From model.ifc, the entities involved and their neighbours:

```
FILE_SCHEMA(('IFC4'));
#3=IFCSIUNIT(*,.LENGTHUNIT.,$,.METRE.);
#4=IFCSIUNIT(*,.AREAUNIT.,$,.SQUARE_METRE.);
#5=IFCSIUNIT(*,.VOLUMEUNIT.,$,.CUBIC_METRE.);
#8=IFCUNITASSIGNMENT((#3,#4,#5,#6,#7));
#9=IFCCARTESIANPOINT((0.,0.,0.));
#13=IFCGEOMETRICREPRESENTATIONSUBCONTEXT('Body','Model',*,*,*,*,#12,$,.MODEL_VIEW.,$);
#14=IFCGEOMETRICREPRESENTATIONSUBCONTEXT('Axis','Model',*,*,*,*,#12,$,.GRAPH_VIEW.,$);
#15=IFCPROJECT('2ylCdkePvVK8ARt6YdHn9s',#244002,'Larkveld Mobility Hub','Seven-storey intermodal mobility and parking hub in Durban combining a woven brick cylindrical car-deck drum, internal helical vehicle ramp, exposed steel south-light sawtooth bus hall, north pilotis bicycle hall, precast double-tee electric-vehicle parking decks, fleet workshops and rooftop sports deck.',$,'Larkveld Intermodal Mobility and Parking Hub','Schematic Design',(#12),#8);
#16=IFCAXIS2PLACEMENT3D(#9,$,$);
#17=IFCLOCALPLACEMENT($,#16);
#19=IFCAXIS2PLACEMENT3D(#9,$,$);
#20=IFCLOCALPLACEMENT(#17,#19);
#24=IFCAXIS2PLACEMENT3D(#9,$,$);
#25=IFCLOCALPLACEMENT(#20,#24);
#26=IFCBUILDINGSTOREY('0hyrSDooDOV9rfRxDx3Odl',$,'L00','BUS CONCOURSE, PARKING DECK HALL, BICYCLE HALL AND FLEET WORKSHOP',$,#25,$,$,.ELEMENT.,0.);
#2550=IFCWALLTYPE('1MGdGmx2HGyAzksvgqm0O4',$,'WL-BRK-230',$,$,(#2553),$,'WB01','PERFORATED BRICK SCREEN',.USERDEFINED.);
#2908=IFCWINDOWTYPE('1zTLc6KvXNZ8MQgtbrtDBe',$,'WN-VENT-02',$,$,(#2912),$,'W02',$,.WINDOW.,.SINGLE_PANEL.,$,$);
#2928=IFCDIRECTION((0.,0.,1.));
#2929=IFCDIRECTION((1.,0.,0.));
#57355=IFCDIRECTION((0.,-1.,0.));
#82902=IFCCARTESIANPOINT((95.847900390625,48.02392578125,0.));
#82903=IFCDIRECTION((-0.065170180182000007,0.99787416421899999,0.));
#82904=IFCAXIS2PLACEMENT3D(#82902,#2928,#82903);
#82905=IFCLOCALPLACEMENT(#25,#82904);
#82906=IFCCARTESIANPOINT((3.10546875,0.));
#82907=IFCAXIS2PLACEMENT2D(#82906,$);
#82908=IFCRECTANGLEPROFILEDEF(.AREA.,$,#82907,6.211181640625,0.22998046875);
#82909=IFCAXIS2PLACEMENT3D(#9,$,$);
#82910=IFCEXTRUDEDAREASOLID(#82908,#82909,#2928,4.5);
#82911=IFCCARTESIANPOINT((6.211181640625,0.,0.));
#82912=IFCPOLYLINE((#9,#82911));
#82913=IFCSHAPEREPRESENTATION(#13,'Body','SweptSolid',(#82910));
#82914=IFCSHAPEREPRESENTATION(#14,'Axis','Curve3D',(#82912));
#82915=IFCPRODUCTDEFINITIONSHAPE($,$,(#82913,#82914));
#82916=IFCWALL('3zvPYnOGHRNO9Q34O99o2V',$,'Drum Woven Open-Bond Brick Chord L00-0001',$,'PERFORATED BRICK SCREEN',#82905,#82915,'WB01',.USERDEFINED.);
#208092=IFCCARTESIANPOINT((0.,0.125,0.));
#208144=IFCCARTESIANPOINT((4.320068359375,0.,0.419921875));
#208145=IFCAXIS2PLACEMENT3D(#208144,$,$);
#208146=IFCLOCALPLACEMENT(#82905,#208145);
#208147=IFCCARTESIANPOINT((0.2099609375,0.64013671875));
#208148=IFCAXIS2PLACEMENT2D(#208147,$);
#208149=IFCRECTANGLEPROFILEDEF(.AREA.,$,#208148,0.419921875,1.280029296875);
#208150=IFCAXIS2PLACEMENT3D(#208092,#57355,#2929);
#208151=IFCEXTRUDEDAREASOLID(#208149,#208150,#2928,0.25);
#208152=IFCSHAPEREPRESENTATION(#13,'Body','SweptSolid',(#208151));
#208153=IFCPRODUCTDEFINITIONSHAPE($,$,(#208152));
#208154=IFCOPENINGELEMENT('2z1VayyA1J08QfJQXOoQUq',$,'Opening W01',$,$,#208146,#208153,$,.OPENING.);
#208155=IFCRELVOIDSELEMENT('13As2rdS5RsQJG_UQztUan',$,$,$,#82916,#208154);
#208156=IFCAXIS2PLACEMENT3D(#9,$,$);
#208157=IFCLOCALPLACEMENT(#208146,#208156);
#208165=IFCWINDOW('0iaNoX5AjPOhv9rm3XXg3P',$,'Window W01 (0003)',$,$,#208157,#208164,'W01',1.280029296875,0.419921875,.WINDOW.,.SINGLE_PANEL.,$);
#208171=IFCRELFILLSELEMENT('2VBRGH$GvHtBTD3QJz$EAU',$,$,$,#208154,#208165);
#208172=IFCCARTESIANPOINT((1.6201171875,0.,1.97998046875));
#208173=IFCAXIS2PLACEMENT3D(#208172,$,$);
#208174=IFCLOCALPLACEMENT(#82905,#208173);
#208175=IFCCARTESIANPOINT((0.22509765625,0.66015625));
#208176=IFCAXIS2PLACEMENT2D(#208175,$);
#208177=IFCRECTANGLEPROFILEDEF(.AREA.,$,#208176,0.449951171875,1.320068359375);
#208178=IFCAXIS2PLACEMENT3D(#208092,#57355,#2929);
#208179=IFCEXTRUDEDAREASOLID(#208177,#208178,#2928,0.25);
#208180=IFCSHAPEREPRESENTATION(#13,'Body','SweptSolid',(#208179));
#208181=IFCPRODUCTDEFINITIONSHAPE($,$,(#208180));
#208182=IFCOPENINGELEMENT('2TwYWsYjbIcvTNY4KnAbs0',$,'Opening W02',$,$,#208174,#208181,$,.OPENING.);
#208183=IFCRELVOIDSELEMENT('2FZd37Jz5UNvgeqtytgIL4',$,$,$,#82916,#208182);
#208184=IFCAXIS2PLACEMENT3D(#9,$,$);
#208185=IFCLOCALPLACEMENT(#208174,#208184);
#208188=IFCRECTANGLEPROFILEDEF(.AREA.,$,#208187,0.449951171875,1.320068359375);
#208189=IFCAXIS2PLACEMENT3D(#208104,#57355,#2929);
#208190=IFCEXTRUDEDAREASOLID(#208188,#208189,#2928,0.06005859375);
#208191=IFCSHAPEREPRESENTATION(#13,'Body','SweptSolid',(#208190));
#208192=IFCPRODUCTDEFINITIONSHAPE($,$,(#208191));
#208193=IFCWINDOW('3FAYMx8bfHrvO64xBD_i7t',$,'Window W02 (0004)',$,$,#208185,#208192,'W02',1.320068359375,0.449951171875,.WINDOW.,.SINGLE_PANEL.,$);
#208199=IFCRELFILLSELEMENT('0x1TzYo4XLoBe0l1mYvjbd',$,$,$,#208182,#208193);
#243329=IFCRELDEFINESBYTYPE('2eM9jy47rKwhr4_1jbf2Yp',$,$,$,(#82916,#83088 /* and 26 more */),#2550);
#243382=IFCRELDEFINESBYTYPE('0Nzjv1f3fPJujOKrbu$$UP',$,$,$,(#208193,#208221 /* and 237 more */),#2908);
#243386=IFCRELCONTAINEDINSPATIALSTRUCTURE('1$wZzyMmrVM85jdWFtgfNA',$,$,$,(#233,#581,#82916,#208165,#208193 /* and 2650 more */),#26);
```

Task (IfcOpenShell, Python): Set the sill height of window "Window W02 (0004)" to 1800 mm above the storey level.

```python
import numpy as np
import ifcopenshell
import ifcopenshell.api.geometry
import ifcopenshell.geom
import ifcopenshell.util.element
import ifcopenshell.util.placement
import ifcopenshell.util.shape
import ifcopenshell.util.unit

model = ifcopenshell.open("model.ifc")
unit_scale = ifcopenshell.util.unit.calculate_unit_scale(model)

window = model.by_guid("3FAYMx8bfHrvO64xBD_i7t")
opening = window.FillsVoids[0].RelatingOpeningElement
storey = ifcopenshell.util.element.get_container(window, ifc_class="IfcBuildingStorey")
level = ifcopenshell.util.placement.get_local_placement(storey.ObjectPlacement)[2, 3]

# The opening's origin need not be at the sill, so measure its lowest point.
shape = ifcopenshell.geom.create_shape(ifcopenshell.geom.settings(), opening)
bottom = ifcopenshell.util.shape.get_shape_bottom_elevation(shape, shape.geometry) / unit_scale
dz = level + 1.8 - bottom

shift = np.array([0.0, 0.0, dz])
# The window is placed relative to its opening, so it follows when the opening moves.
matrix = ifcopenshell.util.placement.get_local_placement(opening.ObjectPlacement)
matrix[:3, 3] += shift
ifcopenshell.api.geometry.edit_object_placement(
    model, product=opening, matrix=matrix, is_si=False, should_transform_children=True
)

print(f"moved by {dz * unit_scale:+.3f} m")

model.write("model-out.ifc")
```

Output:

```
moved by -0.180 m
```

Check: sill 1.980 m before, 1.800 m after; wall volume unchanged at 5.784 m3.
